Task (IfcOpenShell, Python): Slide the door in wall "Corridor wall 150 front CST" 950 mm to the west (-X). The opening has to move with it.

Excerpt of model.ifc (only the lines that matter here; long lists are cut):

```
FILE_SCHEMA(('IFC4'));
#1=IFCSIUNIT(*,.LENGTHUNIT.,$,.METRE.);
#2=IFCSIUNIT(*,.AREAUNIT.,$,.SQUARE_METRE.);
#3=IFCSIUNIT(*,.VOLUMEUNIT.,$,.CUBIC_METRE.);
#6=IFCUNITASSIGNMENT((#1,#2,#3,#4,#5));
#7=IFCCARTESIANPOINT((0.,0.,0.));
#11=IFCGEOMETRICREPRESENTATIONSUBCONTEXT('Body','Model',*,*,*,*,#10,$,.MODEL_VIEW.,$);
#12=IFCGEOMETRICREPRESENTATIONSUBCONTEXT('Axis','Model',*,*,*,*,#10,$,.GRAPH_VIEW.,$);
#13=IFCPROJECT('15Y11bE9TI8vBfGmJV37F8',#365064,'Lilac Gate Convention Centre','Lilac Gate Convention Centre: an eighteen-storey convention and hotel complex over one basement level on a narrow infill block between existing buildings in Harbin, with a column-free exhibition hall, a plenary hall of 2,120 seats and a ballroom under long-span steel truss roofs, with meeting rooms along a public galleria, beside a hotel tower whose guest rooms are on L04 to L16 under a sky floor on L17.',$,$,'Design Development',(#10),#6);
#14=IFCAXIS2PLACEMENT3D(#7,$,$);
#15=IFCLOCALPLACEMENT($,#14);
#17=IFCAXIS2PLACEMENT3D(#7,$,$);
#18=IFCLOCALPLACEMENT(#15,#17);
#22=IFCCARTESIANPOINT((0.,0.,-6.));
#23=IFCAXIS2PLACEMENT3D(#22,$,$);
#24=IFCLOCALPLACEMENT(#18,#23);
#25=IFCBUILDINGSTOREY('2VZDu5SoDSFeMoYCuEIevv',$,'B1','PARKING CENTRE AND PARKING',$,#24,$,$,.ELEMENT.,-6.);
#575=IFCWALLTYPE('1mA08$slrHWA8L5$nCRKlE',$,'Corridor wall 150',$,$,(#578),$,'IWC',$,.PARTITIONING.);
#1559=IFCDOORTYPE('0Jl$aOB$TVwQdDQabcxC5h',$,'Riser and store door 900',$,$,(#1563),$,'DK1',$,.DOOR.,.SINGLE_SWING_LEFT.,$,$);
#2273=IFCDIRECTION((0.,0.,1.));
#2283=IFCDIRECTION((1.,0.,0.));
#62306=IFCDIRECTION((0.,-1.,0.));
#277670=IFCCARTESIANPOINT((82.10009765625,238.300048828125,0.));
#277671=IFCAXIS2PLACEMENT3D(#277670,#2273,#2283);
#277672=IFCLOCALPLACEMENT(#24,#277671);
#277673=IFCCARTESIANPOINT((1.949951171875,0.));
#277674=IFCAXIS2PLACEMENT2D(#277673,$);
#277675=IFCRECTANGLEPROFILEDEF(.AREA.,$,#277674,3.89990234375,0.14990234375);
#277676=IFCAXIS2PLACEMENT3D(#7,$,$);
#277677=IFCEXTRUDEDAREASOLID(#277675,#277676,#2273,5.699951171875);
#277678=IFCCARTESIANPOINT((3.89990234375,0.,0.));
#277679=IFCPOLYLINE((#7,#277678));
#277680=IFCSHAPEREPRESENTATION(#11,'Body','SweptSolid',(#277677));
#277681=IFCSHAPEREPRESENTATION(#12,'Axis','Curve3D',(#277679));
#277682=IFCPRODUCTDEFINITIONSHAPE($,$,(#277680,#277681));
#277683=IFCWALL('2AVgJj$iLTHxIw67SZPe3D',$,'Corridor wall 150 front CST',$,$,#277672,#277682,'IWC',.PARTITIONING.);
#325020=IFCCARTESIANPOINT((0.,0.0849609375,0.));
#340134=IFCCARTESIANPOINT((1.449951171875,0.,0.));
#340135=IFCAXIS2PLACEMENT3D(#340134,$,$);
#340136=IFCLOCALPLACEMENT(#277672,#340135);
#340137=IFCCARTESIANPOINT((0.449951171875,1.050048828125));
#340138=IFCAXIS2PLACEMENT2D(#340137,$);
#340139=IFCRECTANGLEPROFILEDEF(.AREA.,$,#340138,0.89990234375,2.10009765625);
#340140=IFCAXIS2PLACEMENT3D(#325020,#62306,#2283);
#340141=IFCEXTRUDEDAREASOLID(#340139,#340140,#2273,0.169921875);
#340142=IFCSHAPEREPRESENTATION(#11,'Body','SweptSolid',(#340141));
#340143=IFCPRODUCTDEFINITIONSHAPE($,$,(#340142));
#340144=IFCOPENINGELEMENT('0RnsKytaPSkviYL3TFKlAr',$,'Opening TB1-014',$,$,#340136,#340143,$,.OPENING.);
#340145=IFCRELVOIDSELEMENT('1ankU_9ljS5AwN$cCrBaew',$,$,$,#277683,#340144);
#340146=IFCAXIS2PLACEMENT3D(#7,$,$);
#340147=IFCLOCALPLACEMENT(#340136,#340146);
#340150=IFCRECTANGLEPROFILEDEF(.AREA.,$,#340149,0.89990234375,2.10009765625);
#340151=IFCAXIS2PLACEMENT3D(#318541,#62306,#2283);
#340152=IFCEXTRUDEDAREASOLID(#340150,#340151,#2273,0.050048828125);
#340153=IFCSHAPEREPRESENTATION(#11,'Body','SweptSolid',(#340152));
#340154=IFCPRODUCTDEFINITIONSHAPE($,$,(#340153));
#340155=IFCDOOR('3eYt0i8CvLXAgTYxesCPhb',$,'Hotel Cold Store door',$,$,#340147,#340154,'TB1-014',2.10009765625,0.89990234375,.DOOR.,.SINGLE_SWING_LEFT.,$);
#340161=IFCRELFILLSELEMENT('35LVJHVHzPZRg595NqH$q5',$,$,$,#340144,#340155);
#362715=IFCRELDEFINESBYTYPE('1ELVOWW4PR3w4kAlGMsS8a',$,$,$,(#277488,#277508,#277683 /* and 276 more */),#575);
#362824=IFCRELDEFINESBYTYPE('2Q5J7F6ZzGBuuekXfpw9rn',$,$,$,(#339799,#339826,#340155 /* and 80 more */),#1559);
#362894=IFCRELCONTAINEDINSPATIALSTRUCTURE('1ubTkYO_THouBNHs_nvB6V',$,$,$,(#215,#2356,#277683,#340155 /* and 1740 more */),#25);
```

```python
import ifcopenshell
import ifcopenshell.api.geometry
import ifcopenshell.util.placement

model = ifcopenshell.open("model.ifc")

door = model.by_guid("3eYt0i8CvLXAgTYxesCPhb")
opening = door.FillsVoids[0].RelatingOpeningElement
wall = opening.VoidsElements[0].RelatingBuildingElement

wall_matrix = ifcopenshell.util.placement.get_local_placement(wall.ObjectPlacement)
shift = wall_matrix[:3, 0] * -0.95
before = ifcopenshell.util.placement.get_local_placement(door.ObjectPlacement)[:3, 3].copy()

# The door is placed relative to its opening, so it follows when the opening moves.
matrix = ifcopenshell.util.placement.get_local_placement(opening.ObjectPlacement)
matrix[:3, 3] += shift
ifcopenshell.api.geometry.edit_object_placement(
    model, product=opening, matrix=matrix, is_si=False, should_transform_children=True
)

after = ifcopenshell.util.placement.get_local_placement(door.ObjectPlacement)[:3, 3]
print("door moved by", (after - before).round(3) + 0.0)

model.write("model_rev.ifc")
```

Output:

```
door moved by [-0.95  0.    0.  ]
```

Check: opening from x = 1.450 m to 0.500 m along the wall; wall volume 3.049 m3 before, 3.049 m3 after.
